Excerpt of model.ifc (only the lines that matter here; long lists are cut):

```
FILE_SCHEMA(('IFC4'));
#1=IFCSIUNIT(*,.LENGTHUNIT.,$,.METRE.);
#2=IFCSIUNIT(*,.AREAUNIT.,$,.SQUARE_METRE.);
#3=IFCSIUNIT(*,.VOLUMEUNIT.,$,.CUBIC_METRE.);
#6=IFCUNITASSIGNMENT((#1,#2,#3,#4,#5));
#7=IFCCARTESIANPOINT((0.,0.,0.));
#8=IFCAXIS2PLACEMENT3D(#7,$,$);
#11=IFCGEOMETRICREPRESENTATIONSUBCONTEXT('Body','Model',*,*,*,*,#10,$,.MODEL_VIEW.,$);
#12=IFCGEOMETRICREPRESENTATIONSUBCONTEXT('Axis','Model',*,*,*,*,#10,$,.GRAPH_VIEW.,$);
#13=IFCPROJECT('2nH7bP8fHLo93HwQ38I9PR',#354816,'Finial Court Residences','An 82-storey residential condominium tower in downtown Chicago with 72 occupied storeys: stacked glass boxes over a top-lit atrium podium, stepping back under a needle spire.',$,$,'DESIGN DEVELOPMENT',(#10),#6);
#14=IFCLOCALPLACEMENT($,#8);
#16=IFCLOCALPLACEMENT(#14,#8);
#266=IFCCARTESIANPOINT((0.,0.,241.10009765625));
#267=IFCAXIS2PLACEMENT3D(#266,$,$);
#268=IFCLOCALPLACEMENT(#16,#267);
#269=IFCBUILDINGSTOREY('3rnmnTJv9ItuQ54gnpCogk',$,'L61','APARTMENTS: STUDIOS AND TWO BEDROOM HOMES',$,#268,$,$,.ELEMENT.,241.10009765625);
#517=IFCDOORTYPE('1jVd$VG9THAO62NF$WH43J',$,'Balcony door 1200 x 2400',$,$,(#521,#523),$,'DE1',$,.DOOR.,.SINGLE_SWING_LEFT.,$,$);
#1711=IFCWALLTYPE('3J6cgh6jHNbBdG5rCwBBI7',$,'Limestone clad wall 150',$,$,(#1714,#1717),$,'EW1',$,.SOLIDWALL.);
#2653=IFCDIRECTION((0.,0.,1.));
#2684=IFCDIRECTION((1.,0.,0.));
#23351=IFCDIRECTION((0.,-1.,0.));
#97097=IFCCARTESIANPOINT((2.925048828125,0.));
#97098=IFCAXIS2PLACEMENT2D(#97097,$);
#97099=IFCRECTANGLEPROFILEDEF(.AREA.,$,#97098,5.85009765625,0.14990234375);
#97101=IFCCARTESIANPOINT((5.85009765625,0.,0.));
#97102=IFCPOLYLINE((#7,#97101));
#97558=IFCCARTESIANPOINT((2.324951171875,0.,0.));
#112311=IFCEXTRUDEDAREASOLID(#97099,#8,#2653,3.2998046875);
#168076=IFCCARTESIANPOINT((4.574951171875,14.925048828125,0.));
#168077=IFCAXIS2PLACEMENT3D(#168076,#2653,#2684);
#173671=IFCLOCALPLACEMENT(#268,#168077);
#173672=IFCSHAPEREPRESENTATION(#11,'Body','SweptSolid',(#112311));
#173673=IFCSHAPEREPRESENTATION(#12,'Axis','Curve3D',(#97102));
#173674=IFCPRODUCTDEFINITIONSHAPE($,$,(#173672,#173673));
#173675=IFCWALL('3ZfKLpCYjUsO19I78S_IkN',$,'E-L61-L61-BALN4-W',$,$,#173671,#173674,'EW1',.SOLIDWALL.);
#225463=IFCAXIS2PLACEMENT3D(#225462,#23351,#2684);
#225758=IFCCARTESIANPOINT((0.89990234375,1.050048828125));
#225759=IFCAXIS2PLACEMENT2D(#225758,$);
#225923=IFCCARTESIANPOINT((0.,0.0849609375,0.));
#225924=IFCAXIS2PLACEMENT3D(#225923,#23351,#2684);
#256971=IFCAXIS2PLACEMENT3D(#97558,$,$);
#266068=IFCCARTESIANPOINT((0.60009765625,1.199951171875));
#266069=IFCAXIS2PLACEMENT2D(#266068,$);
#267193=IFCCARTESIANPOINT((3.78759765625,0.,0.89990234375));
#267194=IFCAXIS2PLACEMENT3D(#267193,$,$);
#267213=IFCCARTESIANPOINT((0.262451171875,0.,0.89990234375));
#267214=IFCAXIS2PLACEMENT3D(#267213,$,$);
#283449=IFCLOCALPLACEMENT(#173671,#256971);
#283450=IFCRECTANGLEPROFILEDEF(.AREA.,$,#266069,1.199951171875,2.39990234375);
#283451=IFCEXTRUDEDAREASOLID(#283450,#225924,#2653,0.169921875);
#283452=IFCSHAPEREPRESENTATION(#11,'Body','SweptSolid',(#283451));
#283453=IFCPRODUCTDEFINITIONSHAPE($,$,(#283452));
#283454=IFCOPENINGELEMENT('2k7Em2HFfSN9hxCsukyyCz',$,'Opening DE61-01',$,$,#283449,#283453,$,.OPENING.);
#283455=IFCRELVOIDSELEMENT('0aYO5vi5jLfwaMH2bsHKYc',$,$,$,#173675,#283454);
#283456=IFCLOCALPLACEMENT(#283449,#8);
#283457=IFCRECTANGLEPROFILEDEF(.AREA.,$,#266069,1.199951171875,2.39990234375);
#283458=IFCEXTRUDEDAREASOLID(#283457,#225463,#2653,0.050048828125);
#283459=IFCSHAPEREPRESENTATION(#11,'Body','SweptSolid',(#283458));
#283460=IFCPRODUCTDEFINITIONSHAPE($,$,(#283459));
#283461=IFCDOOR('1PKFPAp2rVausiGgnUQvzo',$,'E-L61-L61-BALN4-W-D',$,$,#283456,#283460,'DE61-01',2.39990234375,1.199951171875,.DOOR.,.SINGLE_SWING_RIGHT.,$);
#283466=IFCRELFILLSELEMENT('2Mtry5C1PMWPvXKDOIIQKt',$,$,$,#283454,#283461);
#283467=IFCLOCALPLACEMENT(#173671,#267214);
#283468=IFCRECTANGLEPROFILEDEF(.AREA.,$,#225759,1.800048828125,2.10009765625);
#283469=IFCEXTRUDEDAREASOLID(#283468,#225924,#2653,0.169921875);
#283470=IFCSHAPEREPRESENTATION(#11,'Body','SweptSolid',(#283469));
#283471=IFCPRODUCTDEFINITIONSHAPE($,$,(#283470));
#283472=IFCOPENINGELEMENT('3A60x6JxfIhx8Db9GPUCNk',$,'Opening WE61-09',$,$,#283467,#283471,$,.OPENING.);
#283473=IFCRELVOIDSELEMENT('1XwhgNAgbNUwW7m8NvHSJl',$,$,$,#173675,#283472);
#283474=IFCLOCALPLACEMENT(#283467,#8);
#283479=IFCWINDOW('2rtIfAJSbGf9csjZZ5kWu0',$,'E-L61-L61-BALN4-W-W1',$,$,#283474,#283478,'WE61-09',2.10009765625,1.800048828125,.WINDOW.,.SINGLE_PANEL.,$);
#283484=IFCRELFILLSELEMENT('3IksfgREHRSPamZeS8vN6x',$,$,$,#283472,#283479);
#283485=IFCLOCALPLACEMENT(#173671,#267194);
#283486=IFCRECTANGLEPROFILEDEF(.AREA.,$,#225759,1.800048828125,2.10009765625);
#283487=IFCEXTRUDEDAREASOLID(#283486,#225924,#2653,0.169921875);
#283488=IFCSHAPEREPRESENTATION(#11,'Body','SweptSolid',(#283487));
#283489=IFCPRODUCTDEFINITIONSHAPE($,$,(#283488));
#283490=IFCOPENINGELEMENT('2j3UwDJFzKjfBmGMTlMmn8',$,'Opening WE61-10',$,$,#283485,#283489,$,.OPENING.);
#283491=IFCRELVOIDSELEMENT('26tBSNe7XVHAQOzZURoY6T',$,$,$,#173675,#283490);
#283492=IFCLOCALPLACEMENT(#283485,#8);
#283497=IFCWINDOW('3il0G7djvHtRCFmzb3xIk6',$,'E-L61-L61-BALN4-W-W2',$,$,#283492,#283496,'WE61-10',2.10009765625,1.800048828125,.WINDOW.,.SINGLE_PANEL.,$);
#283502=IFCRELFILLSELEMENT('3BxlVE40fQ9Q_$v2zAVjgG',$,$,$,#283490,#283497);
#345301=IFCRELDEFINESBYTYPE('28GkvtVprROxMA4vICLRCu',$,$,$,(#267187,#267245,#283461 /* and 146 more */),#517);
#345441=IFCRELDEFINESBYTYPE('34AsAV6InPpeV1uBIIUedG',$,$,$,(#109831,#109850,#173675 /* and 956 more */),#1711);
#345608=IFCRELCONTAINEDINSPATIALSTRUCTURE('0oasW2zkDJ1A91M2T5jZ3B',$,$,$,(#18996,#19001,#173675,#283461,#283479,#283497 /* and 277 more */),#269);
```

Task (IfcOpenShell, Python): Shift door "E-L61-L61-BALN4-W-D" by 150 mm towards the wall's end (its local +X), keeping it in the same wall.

```python
import ifcopenshell
import ifcopenshell.api.geometry
import ifcopenshell.util.placement

model = ifcopenshell.open("model.ifc")

door = model.by_id(283461)
opening = door.FillsVoids[0].RelatingOpeningElement
wall = opening.VoidsElements[0].RelatingBuildingElement

wall_matrix = ifcopenshell.util.placement.get_local_placement(wall.ObjectPlacement)
shift = wall_matrix[:3, 0] * 0.15
before = ifcopenshell.util.placement.get_local_placement(door.ObjectPlacement)[:3, 3].copy()

# The door is placed relative to its opening, so it follows when the opening moves.
matrix = ifcopenshell.util.placement.get_local_placement(opening.ObjectPlacement)
matrix[:3, 3] += shift
ifcopenshell.api.geometry.edit_object_placement(
    model, product=opening, matrix=matrix, is_si=False, should_transform_children=True
)

after = ifcopenshell.util.placement.get_local_placement(door.ObjectPlacement)[:3, 3]
print("door moved by", (after - before).round(3) + 0.0)

model.write("model_v2.ifc")
```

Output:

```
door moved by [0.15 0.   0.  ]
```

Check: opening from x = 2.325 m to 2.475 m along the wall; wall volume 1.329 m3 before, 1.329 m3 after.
